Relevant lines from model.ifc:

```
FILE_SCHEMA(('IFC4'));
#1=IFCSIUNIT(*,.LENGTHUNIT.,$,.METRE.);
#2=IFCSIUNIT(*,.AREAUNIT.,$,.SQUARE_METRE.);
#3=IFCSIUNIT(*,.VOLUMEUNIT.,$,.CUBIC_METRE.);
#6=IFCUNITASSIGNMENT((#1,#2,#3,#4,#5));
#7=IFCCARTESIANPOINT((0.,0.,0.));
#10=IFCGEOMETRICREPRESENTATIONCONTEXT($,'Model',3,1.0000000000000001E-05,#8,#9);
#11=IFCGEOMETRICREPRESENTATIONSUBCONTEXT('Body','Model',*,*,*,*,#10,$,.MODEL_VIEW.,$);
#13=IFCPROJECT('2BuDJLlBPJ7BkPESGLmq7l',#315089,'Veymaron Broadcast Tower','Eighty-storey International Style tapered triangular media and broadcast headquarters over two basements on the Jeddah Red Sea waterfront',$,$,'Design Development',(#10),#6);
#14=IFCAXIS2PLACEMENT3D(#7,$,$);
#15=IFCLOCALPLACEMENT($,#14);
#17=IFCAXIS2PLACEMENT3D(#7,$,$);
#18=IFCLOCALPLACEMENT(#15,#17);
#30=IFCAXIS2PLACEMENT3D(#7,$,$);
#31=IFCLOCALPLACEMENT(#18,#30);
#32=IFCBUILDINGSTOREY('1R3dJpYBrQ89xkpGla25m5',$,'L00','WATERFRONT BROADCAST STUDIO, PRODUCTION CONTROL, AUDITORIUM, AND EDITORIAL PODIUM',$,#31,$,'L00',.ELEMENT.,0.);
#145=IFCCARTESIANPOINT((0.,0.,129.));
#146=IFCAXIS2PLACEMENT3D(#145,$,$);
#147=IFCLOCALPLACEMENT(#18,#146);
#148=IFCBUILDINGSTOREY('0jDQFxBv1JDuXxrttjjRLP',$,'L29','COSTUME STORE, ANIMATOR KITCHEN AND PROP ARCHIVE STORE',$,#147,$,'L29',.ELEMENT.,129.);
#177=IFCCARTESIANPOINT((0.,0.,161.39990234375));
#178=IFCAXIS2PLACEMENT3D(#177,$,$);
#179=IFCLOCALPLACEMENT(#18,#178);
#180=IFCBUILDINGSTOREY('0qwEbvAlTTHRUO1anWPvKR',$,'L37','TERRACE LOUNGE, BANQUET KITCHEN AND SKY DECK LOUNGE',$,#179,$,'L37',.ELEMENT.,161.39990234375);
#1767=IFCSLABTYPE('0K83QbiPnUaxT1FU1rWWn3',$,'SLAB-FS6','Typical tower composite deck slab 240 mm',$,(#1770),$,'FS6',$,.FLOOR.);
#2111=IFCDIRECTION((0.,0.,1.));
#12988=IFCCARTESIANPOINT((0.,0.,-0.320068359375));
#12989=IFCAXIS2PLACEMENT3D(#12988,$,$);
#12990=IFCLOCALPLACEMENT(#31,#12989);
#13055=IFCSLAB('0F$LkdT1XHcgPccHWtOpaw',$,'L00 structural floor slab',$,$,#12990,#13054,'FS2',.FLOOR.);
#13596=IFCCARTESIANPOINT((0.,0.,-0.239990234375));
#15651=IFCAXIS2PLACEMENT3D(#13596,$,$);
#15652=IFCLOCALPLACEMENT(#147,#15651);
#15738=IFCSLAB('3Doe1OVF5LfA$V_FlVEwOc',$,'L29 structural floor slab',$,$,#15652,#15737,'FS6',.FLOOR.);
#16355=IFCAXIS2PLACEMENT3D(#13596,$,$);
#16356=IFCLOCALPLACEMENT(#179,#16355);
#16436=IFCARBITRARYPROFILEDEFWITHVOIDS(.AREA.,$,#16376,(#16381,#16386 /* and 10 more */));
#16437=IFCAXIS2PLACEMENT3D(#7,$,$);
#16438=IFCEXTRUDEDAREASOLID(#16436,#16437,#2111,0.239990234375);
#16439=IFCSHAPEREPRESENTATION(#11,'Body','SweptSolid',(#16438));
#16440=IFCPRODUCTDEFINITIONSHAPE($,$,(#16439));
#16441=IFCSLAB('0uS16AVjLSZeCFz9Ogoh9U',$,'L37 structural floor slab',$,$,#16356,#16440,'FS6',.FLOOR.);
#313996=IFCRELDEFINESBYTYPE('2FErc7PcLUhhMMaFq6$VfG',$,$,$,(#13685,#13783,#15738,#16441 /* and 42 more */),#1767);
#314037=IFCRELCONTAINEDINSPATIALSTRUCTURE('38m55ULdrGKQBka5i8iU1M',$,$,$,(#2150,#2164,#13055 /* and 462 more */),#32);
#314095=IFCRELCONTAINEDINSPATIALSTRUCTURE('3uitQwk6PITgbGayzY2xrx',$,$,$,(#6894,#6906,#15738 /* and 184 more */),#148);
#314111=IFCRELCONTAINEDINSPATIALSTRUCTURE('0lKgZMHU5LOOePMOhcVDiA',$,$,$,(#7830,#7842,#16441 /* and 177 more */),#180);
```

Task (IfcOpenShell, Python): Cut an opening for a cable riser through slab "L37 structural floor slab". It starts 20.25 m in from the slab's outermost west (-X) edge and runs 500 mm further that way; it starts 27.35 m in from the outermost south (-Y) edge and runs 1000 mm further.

```python
import numpy as np
import ifcopenshell
import ifcopenshell.api.feature
import ifcopenshell.api.geometry
import ifcopenshell.api.root
import ifcopenshell.geom
import ifcopenshell.util.placement
import ifcopenshell.util.representation
import ifcopenshell.util.shape
import ifcopenshell.util.unit

model = ifcopenshell.open("model.ifc")
unit_scale = ifcopenshell.util.unit.calculate_unit_scale(model)
settings = ifcopenshell.geom.settings()


def volume(element):
    """Net volume in cubic metres, openings subtracted."""
    shape = ifcopenshell.geom.create_shape(settings, element)
    return ifcopenshell.util.shape.get_volume(shape.geometry)


slab = model.by_guid("0uS16AVjLSZeCFz9Ogoh9U")
before = volume(slab)

# Extent in the slab's own axes, in metres. The edges named are its -X and -Y sides.
slab_shape = ifcopenshell.geom.create_shape(settings, slab)
vertices = ifcopenshell.util.shape.get_vertices(slab_shape.geometry)
x_min, y_min, bottom = vertices.min(axis=0)
top = vertices[:, 2].max()

opening = ifcopenshell.api.root.create_entity(model, ifc_class="IfcOpeningElement", name="Cable riser opening", predefined_type="OPENING")
context = ifcopenshell.util.representation.get_context(model, "Model", "Body", "MODEL_VIEW")
width, depth = 0.5, 1
outline = [(0.0, 0.0), (width, 0.0), (width, depth), (0.0, depth), (0.0, 0.0)]
# Overshoot both faces by 50 mm so the cut is clean.
shape = ifcopenshell.api.geometry.add_slab_representation(
    model, context=context, depth=top - bottom + 0.1, polyline=outline
)
ifcopenshell.api.geometry.assign_representation(model, product=opening, representation=shape)

matrix = ifcopenshell.util.placement.get_local_placement(slab.ObjectPlacement)
matrix[:, 3] = matrix @ np.append(np.array([x_min + 20.25, y_min + 27.35, bottom - 0.05]) / unit_scale, 1.0)
ifcopenshell.api.geometry.edit_object_placement(model, product=opening, matrix=matrix, is_si=False)
ifcopenshell.api.feature.add_feature(model, feature=opening, element=slab)

after = volume(slab)

print(f"slab volume {before:.3f} -> {after:.3f} m3")

model.write("model-out.ifc")
```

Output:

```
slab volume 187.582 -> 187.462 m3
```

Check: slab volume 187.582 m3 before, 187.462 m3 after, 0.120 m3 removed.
